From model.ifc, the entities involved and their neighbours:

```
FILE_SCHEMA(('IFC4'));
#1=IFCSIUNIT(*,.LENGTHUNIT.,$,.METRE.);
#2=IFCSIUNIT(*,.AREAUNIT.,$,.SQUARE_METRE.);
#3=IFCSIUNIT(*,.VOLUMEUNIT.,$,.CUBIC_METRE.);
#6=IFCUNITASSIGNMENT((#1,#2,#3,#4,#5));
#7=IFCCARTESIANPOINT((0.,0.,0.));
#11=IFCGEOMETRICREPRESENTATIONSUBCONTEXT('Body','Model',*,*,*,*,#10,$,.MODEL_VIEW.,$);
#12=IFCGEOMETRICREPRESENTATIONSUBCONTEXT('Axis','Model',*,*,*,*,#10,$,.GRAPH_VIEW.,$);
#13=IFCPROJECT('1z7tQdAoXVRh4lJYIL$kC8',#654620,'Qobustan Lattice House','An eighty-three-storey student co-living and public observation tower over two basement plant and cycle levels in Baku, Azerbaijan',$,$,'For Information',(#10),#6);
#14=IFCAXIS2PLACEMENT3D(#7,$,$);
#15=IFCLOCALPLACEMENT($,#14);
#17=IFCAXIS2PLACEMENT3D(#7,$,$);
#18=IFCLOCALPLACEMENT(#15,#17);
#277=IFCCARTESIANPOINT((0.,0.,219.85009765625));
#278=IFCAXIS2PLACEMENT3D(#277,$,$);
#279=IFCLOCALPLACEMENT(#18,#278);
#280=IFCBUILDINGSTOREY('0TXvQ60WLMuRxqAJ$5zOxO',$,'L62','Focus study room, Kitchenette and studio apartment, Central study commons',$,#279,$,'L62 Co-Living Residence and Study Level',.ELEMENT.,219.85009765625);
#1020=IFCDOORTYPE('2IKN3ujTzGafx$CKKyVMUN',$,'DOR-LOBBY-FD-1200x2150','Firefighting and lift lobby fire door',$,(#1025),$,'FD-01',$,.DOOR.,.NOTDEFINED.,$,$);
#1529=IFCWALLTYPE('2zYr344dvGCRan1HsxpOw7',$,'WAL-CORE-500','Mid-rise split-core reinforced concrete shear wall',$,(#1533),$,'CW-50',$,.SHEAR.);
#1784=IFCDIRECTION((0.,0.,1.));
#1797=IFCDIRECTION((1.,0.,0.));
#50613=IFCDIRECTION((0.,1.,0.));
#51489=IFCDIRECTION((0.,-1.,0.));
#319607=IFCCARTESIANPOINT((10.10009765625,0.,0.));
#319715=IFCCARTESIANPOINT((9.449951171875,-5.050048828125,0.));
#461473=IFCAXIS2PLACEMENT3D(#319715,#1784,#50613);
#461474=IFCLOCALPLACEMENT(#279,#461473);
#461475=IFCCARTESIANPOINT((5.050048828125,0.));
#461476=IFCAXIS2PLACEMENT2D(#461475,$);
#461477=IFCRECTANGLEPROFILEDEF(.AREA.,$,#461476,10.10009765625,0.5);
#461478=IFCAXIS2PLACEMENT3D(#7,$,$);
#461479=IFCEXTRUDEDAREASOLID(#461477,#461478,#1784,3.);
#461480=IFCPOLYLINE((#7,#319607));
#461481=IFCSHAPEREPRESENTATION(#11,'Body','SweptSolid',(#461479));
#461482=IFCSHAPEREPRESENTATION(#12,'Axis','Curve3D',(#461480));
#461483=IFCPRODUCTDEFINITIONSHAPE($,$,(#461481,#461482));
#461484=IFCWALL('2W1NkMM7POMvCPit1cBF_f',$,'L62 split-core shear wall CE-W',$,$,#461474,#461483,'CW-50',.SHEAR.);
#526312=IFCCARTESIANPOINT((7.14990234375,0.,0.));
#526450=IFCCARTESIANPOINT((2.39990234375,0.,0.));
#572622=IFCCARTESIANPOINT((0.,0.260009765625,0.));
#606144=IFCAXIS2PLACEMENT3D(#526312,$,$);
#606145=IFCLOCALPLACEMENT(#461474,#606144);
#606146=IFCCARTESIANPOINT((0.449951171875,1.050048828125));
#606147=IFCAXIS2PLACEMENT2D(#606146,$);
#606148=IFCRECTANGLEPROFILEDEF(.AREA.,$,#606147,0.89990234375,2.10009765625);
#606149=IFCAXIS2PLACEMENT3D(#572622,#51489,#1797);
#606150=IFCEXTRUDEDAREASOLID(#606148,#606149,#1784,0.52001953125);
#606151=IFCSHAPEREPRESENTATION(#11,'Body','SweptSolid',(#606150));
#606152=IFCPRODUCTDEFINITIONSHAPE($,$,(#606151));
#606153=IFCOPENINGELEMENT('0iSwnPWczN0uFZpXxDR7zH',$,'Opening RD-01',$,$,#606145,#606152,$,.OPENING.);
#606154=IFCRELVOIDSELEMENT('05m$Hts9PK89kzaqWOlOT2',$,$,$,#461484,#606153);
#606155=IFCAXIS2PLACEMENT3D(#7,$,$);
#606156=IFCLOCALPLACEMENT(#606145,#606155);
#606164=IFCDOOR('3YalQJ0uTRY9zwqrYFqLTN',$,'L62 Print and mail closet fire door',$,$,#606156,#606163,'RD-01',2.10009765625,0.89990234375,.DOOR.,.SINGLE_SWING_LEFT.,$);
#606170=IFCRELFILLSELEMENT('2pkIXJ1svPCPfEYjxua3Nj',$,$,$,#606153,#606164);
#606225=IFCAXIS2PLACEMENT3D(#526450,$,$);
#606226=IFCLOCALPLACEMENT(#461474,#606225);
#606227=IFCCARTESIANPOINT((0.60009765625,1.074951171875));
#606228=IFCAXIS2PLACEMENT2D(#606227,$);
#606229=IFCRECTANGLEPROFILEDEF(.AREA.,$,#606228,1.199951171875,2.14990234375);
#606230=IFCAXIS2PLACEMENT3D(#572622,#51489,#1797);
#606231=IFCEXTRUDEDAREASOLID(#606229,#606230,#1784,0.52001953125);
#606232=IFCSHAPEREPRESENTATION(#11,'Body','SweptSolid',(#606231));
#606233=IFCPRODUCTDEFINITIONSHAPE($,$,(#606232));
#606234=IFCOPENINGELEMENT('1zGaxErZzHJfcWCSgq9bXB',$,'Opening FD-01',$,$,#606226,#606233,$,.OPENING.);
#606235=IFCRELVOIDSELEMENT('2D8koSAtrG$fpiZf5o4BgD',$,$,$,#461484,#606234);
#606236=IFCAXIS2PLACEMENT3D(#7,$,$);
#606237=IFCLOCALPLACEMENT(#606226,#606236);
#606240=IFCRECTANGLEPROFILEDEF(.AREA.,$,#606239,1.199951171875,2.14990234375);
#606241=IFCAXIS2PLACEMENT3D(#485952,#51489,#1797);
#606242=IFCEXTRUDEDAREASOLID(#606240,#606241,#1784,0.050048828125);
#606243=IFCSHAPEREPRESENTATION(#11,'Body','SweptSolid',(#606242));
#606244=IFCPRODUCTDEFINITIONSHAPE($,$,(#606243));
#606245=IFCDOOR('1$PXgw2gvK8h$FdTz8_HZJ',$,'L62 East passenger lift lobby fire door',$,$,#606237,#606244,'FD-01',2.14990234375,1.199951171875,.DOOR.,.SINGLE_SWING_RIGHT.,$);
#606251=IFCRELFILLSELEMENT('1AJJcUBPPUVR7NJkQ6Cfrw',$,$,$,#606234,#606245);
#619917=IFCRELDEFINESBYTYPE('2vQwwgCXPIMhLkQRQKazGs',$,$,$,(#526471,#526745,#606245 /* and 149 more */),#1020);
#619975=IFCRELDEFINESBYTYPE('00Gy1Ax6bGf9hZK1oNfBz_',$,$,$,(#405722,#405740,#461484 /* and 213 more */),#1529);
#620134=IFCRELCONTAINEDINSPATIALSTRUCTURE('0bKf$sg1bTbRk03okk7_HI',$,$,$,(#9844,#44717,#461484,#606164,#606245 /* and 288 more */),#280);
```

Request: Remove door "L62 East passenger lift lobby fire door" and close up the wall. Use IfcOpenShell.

```python
import ifcopenshell
import ifcopenshell.api.feature
import ifcopenshell.api.root
import ifcopenshell.geom
import ifcopenshell.util.shape

model = ifcopenshell.open("model.ifc")
settings = ifcopenshell.geom.settings()


def volume(element):
    """Net volume in cubic metres, openings subtracted."""
    shape = ifcopenshell.geom.create_shape(settings, element)
    return ifcopenshell.util.shape.get_volume(shape.geometry)


door = model.by_guid("1$PXgw2gvK8h$FdTz8_HZJ")
opening = door.FillsVoids[0].RelatingOpeningElement
wall = opening.VoidsElements[0].RelatingBuildingElement
before = volume(wall)

ifcopenshell.api.root.remove_product(model, product=door)
ifcopenshell.api.feature.remove_feature(model, feature=opening)

after = volume(wall)

print(f"wall volume {before:.3f} -> {after:.3f} m3")

model.write("model_v2.ifc")
```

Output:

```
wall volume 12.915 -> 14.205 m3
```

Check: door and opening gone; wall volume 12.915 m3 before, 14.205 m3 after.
